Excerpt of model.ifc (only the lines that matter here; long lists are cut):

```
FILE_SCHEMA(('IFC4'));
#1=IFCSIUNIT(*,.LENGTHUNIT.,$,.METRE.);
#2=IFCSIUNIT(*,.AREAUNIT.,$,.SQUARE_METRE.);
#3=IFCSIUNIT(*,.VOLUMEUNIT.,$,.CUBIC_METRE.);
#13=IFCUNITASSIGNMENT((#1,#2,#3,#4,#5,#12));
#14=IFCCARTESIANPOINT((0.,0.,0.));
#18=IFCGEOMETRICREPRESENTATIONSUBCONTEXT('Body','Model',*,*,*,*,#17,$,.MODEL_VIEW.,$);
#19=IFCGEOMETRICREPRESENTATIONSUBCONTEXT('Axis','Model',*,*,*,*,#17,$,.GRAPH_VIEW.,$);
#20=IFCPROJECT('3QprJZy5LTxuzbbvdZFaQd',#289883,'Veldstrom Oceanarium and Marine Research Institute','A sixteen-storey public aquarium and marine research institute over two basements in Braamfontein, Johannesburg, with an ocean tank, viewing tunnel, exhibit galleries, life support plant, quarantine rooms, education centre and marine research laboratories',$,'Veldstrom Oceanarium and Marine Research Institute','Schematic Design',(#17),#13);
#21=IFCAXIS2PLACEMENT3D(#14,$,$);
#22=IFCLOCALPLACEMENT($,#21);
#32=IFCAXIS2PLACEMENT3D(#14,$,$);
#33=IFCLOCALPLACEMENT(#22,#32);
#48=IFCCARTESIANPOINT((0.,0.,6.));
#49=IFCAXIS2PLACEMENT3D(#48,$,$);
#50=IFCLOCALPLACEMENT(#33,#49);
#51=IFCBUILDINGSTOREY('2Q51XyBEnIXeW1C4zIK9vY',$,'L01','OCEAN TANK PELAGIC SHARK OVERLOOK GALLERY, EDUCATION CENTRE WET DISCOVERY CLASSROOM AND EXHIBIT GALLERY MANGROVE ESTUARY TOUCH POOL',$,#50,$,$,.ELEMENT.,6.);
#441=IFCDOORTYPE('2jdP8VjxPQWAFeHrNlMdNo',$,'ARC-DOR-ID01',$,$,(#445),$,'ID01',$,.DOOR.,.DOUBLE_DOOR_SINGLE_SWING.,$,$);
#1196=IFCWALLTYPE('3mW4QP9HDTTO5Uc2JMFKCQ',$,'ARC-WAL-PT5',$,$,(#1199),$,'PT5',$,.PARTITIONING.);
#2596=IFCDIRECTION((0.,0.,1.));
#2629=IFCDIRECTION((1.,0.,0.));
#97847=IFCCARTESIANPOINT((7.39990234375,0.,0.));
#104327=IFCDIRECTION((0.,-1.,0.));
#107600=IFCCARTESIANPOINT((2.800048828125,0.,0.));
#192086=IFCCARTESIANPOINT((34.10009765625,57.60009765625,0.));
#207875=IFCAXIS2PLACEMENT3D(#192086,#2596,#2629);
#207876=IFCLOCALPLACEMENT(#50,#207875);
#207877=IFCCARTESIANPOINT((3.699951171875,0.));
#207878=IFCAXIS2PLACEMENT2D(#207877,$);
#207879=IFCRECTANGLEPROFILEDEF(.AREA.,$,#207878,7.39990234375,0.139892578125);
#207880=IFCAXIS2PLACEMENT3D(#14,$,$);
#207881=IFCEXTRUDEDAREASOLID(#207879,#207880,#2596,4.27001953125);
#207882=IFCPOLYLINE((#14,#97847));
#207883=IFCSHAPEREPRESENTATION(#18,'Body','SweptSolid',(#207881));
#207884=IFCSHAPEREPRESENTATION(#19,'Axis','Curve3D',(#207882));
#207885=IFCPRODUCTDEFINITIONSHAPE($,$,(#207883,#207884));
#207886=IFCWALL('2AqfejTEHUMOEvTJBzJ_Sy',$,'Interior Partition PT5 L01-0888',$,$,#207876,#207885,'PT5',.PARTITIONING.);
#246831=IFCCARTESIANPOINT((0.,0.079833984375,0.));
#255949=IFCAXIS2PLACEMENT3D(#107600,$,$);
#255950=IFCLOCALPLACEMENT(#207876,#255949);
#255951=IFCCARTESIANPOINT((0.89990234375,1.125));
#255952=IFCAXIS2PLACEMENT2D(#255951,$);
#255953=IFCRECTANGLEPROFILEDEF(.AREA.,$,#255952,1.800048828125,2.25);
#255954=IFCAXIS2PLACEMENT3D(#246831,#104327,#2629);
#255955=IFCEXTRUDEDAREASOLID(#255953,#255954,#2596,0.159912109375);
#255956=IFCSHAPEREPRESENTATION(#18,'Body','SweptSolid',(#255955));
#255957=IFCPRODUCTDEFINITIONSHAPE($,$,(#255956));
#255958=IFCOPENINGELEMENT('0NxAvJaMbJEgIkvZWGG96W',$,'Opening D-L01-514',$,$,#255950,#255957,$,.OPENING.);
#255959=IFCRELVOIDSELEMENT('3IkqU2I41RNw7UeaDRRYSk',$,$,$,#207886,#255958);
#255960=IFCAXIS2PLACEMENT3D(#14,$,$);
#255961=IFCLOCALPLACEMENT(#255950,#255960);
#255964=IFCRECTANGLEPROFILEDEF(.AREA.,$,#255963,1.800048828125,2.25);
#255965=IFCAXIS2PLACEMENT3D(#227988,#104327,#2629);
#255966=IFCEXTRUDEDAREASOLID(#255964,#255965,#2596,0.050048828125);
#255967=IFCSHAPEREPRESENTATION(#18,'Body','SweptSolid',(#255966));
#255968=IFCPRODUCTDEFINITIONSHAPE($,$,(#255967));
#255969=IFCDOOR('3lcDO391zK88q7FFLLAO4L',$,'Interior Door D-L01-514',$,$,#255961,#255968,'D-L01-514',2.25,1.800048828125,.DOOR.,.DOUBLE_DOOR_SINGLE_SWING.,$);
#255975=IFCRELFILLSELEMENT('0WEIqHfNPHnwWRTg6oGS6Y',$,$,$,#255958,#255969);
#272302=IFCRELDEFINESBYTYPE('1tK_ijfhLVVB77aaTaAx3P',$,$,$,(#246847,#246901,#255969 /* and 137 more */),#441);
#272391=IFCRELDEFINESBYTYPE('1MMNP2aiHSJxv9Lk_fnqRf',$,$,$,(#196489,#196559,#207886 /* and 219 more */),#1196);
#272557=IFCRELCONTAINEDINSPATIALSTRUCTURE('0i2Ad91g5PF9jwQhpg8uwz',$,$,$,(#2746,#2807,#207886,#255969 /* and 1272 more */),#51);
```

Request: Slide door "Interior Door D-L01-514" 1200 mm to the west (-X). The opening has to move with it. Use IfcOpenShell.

```python
import ifcopenshell
import ifcopenshell.api.geometry
import ifcopenshell.util.placement
import ifcopenshell.util.unit

model = ifcopenshell.open("model.ifc")
unit_scale = ifcopenshell.util.unit.calculate_unit_scale(model)

door = model.by_guid("3lcDO391zK88q7FFLLAO4L")
opening = door.FillsVoids[0].RelatingOpeningElement
wall = opening.VoidsElements[0].RelatingBuildingElement

wall_matrix = ifcopenshell.util.placement.get_local_placement(wall.ObjectPlacement)
shift = wall_matrix[:3, 0] * -1.2 / unit_scale
before = ifcopenshell.util.placement.get_local_placement(door.ObjectPlacement)[:3, 3].copy()

# The door is placed relative to its opening, so it follows when the opening moves.
matrix = ifcopenshell.util.placement.get_local_placement(opening.ObjectPlacement)
matrix[:3, 3] += shift
ifcopenshell.api.geometry.edit_object_placement(
    model, product=opening, matrix=matrix, is_si=False, should_transform_children=True
)

after = ifcopenshell.util.placement.get_local_placement(door.ObjectPlacement)[:3, 3]
print("door moved by", (after - before).round(3) + 0.0)

model.write("model_v2.ifc")
```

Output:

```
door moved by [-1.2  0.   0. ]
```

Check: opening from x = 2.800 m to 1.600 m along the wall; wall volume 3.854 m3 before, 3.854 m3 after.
